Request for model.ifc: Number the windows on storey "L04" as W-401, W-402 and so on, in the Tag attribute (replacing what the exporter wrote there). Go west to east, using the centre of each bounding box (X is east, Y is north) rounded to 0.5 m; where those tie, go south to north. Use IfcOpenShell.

First a look at what the model holds.

```python
import ifcopenshell
import ifcopenshell.util.element
import ifcopenshell.util.placement

model = ifcopenshell.open("model.ifc")
print(model.schema)
storey = next(s for s in model.by_type("IfcBuildingStorey") if s.Name == "L04")
windows = [e for e in ifcopenshell.util.element.get_decomposition(storey) if e.is_a("IfcWindow")]
for e in sorted(windows, key=lambda e: e.id()):
    origin = ifcopenshell.util.placement.get_local_placement(e.ObjectPlacement)[:3, 3]
    print(e.id(), e.Tag, e.Name, origin.round(2) + 0.0, sep=" | ")
```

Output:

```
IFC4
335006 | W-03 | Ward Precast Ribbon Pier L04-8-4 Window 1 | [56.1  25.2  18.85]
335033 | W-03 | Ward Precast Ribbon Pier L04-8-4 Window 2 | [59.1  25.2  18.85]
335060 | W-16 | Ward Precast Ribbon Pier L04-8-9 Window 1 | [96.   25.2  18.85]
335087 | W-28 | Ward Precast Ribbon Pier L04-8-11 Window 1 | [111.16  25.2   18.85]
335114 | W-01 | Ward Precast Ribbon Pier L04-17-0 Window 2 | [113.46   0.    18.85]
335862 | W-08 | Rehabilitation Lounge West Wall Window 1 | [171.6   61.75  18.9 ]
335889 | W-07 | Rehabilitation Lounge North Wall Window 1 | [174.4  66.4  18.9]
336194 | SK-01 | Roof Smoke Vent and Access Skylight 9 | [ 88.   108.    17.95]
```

```python
import ifcopenshell
import ifcopenshell.geom
import ifcopenshell.util.element
import ifcopenshell.util.shape

model = ifcopenshell.open("model.ifc")
settings = ifcopenshell.geom.settings()
settings.set("use-world-coords", True)


def centre(element):
    shape = ifcopenshell.geom.create_shape(settings, element)
    return ifcopenshell.util.shape.get_bbox_centroid(shape.geometry)


storey = next(s for s in model.by_type("IfcBuildingStorey") if s.Name == "L04")
windows = [e for e in ifcopenshell.util.element.get_decomposition(storey) if e.is_a("IfcWindow")]

# Insertion points can sit at a corner or the storey origin, so sort by the geometry (in metres).
centres = {e: centre(e) for e in windows}
windows.sort(key=lambda e: (round(centres[e][0] / 0.5), centres[e][1]))

for i, e in enumerate(windows, start=1):
    number = f"W-4{i:02d}"
    e.Tag = number
    print(e.id(), number)

model.write("model_updated.ifc")
```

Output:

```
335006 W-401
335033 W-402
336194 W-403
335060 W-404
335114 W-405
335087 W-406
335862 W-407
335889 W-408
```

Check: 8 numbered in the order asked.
